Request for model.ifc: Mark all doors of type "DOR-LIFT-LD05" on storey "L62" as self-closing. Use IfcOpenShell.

First a look at what the model holds.

```python
import ifcopenshell
import ifcopenshell.util.element

model = ifcopenshell.open("model.ifc")
print(model.schema)
storey = next(s for s in model.by_type("IfcBuildingStorey") if s.Name == "L62")
doors = [e for e in ifcopenshell.util.element.get_decomposition(storey) if e.is_a("IfcDoor")]
seen = {}
for e in doors:
    element_type = ifcopenshell.util.element.get_type(e)
    key = (element_type.Name if element_type != e and element_type else None, ifcopenshell.util.element.get_pset(e, "Pset_DoorCommon", "SelfClosing"))
    seen[key] = seen.get(key, 0) + 1
for (name, value), count in sorted(seen.items(), key=str):
    print(count, "x", name, "|", value)
```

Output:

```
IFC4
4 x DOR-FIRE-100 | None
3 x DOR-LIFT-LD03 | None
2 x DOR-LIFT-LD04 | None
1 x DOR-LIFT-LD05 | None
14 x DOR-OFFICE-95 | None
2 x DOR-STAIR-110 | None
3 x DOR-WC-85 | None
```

```python
import ifcopenshell
import ifcopenshell.api.pset
import ifcopenshell.util.element

model = ifcopenshell.open("model.ifc")

storey = next(s for s in model.by_type("IfcBuildingStorey") if s.Name == "L62")
doors = [e for e in ifcopenshell.util.element.get_decomposition(storey) if e.is_a("IfcDoor")]

count = 0
for e in doors:
    element_type = ifcopenshell.util.element.get_type(e)
    if element_type in (None, e) or element_type.Name != "DOR-LIFT-LD05":
        continue
    found = ifcopenshell.util.element.get_pset(e, "Pset_DoorCommon", should_inherit=False)
    if found:
        pset = model.by_id(found["id"])
        if len(ifcopenshell.util.element.get_elements_by_pset(pset)) > 1:
            pset = ifcopenshell.api.pset.unshare_pset(model, products=[e], pset=pset)[0]
    else:
        pset = ifcopenshell.api.pset.add_pset(model, product=e, name="Pset_DoorCommon")
    ifcopenshell.api.pset.edit_pset(model, pset=pset, properties={"SelfClosing": True})
    count += 1

print(count, "doors updated")

model.write("model_updated.ifc")
```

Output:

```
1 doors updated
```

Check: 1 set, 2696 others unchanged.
